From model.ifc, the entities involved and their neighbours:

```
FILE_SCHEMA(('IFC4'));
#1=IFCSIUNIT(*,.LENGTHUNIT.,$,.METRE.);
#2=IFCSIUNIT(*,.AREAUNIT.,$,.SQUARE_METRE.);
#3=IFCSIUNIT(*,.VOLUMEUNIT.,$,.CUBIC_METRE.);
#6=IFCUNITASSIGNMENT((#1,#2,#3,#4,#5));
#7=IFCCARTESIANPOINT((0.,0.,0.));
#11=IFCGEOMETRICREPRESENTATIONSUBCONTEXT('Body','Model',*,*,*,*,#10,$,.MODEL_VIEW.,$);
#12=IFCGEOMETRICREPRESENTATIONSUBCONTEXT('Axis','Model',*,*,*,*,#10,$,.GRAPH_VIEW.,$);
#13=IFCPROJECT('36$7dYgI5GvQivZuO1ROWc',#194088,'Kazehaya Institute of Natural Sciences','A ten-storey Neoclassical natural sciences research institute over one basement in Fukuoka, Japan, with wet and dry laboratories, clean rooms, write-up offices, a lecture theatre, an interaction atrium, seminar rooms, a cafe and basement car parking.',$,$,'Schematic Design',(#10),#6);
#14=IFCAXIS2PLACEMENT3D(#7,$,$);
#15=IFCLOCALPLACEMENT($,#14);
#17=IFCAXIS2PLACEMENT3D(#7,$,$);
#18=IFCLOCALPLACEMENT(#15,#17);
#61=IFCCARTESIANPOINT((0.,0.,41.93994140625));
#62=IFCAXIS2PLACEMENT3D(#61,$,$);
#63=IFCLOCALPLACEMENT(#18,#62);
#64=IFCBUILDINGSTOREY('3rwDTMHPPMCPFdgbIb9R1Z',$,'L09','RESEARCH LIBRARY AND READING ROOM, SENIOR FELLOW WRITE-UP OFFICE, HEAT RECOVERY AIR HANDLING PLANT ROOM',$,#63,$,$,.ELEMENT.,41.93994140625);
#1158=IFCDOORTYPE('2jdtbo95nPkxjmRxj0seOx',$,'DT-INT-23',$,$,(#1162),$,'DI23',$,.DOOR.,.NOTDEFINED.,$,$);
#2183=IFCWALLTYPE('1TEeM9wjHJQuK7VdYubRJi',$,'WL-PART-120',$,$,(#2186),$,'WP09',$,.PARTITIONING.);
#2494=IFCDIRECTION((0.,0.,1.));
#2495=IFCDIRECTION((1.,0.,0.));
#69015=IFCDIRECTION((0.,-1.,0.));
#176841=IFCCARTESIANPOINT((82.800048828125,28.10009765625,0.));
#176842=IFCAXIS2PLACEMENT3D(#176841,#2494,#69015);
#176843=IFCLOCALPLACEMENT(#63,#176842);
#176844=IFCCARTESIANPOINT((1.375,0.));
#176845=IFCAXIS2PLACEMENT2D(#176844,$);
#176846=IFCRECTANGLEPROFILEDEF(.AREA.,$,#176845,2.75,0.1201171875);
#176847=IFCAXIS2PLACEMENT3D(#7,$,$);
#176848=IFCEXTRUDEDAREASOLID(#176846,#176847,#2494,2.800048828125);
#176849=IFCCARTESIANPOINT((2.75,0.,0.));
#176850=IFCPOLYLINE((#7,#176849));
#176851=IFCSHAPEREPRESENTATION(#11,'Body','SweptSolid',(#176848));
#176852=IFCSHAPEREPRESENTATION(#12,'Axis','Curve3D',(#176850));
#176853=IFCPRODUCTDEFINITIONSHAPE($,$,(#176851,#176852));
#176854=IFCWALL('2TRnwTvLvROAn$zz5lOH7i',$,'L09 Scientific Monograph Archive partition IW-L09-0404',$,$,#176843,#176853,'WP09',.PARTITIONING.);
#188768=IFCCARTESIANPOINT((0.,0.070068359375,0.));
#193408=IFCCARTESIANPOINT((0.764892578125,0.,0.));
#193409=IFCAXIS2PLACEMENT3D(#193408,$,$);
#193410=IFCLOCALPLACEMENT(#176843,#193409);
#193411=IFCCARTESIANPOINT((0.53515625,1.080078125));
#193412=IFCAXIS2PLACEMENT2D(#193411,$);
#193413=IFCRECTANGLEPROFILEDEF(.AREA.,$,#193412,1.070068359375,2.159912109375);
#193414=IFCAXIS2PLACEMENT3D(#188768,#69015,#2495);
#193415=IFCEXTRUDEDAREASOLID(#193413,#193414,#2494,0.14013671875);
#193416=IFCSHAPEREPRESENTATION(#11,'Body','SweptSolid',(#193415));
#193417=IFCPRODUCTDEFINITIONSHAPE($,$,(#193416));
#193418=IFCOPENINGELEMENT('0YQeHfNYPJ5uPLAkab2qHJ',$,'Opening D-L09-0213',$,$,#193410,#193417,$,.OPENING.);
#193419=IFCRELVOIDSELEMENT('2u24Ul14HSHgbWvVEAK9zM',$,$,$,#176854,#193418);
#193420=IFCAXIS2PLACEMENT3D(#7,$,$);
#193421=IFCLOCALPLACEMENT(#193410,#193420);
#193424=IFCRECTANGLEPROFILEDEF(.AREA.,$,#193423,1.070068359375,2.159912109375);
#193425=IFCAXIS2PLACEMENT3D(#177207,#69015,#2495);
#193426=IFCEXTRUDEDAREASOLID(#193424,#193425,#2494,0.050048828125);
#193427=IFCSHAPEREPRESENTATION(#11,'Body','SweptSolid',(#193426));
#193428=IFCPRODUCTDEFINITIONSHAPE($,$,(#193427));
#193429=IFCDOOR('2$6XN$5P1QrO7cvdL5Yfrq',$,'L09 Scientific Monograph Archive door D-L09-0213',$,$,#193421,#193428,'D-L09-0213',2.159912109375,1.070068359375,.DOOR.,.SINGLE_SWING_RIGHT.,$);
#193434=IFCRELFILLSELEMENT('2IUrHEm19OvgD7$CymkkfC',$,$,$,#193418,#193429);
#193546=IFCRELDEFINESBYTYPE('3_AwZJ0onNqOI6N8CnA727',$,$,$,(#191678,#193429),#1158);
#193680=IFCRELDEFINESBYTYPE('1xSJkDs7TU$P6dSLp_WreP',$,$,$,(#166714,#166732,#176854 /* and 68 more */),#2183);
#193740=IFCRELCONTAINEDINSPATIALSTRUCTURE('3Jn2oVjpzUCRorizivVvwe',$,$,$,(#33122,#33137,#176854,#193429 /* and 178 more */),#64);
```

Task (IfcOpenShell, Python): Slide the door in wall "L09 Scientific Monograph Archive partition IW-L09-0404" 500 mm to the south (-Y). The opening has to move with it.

```python
import ifcopenshell
import ifcopenshell.api.geometry
import ifcopenshell.util.placement

model = ifcopenshell.open("model.ifc")

door = model.by_guid("2$6XN$5P1QrO7cvdL5Yfrq")
opening = door.FillsVoids[0].RelatingOpeningElement
wall = opening.VoidsElements[0].RelatingBuildingElement

wall_matrix = ifcopenshell.util.placement.get_local_placement(wall.ObjectPlacement)
shift = wall_matrix[:3, 0] * 0.5
before = ifcopenshell.util.placement.get_local_placement(door.ObjectPlacement)[:3, 3].copy()

# The door is placed relative to its opening, so it follows when the opening moves.
matrix = ifcopenshell.util.placement.get_local_placement(opening.ObjectPlacement)
matrix[:3, 3] += shift
ifcopenshell.api.geometry.edit_object_placement(
    model, product=opening, matrix=matrix, is_si=False, should_transform_children=True
)

after = ifcopenshell.util.placement.get_local_placement(door.ObjectPlacement)[:3, 3]
print("door moved by", (after - before).round(3) + 0.0)

model.write("model_v2.ifc")
```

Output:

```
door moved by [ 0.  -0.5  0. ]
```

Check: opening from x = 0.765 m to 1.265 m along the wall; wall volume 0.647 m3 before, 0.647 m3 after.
